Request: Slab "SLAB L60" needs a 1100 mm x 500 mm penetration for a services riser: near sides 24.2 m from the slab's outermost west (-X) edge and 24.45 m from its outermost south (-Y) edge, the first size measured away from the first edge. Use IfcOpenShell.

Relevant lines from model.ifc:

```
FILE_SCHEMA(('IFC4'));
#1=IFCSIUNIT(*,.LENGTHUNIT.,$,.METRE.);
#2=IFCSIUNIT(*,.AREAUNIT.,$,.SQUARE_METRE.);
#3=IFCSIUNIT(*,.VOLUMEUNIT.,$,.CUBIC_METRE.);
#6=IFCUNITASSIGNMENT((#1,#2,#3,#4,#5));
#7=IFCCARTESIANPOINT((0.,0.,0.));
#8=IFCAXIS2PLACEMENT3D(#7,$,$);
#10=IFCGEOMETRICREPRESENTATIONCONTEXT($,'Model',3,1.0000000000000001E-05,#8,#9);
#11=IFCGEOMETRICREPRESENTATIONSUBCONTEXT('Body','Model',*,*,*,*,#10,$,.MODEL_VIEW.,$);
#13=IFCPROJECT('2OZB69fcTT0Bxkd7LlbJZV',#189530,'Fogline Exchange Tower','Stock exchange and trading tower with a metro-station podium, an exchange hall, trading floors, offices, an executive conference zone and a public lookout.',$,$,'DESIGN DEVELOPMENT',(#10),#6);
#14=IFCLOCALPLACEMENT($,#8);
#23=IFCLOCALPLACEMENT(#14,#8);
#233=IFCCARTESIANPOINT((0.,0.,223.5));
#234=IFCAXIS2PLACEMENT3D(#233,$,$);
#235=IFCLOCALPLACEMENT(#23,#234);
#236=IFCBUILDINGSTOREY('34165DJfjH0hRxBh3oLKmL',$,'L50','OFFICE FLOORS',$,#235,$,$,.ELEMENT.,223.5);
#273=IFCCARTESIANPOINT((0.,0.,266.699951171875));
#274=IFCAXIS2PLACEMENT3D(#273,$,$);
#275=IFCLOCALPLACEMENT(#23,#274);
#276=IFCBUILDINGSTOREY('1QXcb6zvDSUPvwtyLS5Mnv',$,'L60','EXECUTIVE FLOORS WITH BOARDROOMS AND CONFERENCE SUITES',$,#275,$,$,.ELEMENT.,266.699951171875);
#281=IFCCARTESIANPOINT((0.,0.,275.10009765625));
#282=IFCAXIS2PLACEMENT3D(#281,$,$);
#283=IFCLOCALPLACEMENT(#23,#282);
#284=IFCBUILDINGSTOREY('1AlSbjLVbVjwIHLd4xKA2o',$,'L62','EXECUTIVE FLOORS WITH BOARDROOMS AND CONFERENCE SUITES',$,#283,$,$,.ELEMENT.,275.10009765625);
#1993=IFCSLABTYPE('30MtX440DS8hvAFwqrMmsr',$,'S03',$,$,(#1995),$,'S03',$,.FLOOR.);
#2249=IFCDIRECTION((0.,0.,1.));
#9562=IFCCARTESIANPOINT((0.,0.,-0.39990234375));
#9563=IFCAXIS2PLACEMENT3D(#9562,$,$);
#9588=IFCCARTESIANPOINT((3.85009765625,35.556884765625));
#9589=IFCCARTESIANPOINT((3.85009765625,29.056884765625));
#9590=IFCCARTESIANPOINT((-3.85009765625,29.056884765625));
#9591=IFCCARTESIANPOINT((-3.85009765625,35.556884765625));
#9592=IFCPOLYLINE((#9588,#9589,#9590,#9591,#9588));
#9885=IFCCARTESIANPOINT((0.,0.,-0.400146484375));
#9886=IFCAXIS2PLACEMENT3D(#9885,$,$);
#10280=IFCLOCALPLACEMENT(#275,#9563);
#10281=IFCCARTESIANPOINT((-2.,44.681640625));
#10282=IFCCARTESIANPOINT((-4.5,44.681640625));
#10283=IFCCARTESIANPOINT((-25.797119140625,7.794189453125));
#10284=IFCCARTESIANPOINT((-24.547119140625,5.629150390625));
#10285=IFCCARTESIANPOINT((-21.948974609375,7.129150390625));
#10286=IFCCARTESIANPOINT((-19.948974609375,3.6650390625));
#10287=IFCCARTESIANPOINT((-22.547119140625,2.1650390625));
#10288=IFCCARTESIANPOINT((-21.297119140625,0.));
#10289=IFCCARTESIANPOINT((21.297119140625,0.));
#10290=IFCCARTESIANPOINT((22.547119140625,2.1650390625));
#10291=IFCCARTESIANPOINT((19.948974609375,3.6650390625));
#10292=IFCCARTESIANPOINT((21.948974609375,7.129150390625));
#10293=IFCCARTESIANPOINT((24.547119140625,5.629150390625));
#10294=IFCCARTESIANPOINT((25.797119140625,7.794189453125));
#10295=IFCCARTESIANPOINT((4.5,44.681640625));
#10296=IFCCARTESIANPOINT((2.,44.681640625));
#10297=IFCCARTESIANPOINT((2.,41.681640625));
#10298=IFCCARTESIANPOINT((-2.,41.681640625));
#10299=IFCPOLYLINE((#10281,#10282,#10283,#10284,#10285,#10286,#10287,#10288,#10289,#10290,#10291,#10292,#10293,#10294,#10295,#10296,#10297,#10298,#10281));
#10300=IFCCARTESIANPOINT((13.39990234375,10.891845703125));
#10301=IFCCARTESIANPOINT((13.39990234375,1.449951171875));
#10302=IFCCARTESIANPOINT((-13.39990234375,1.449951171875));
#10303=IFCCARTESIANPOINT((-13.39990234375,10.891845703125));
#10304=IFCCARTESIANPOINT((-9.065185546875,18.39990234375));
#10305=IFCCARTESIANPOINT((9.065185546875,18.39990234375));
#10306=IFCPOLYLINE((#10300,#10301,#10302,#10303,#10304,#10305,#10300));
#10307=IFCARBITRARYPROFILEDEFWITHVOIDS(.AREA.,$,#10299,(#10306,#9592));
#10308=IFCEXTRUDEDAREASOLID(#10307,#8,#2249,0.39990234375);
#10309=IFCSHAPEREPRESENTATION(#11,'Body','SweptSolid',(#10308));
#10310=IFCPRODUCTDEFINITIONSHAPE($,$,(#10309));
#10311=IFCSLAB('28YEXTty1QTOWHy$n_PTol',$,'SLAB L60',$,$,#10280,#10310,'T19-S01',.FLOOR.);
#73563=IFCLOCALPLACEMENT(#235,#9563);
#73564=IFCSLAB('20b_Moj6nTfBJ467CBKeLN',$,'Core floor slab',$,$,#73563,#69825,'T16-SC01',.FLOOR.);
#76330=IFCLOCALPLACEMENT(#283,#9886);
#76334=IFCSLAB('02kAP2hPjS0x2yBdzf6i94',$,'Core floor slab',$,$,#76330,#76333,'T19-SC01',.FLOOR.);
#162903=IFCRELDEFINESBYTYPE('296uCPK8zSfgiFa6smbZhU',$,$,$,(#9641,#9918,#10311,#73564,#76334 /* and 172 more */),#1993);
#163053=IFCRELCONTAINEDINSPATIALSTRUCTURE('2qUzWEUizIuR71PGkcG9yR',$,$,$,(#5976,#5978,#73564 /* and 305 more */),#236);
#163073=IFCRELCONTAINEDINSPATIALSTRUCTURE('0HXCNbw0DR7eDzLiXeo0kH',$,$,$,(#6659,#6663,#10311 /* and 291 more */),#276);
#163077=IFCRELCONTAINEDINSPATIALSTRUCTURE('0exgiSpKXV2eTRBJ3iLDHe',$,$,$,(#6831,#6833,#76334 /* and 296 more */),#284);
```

```python
import numpy as np
import ifcopenshell
import ifcopenshell.api.feature
import ifcopenshell.api.geometry
import ifcopenshell.api.root
import ifcopenshell.geom
import ifcopenshell.util.placement
import ifcopenshell.util.representation
import ifcopenshell.util.shape
import ifcopenshell.util.unit

model = ifcopenshell.open("model.ifc")
unit_scale = ifcopenshell.util.unit.calculate_unit_scale(model)
settings = ifcopenshell.geom.settings()


def volume(element):
    """Net volume in cubic metres, openings subtracted."""
    shape = ifcopenshell.geom.create_shape(settings, element)
    return ifcopenshell.util.shape.get_volume(shape.geometry)


slab = model.by_id(10311)
before = volume(slab)

# Extent in the slab's own axes, in metres. The edges named are its -X and -Y sides.
slab_shape = ifcopenshell.geom.create_shape(settings, slab)
vertices = ifcopenshell.util.shape.get_vertices(slab_shape.geometry)
x_min, y_min, bottom = vertices.min(axis=0)
top = vertices[:, 2].max()

opening = ifcopenshell.api.root.create_entity(model, ifc_class="IfcOpeningElement", name="Services riser opening", predefined_type="OPENING")
context = ifcopenshell.util.representation.get_context(model, "Model", "Body", "MODEL_VIEW")
width, depth = 1.1, 0.5
outline = [(0.0, 0.0), (width, 0.0), (width, depth), (0.0, depth), (0.0, 0.0)]
# Overshoot both faces by 50 mm so the cut is clean.
shape = ifcopenshell.api.geometry.add_slab_representation(
    model, context=context, depth=top - bottom + 0.1, polyline=outline
)
ifcopenshell.api.geometry.assign_representation(model, product=opening, representation=shape)

matrix = ifcopenshell.util.placement.get_local_placement(slab.ObjectPlacement)
matrix[:, 3] = matrix @ np.append(np.array([x_min + 24.2, y_min + 24.45, bottom - 0.05]) / unit_scale, 1.0)
ifcopenshell.api.geometry.edit_object_placement(model, product=opening, matrix=matrix, is_si=False)
ifcopenshell.api.feature.add_feature(model, feature=opening, element=slab)

after = volume(slab)

print(f"slab volume {before:.3f} -> {after:.3f} m3")

model.write("model_rev.ifc")
```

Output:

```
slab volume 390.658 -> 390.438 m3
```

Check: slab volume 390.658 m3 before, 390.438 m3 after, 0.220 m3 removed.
